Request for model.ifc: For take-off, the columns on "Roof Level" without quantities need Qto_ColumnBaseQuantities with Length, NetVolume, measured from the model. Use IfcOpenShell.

First a look at what the model holds.

```python
import ifcopenshell
import ifcopenshell.util.element
import ifcopenshell.util.unit

model = ifcopenshell.open("model.ifc")
print(model.schema)
for unit_type in ("LENGTHUNIT", "AREAUNIT", "VOLUMEUNIT"):
    print(unit_type, ifcopenshell.util.unit.calculate_unit_scale(model, unit_type))
storey = next(s for s in model.by_type("IfcBuildingStorey") if s.Name == "Roof Level")
columns = [e for e in ifcopenshell.util.element.get_decomposition(storey) if e.is_a("IfcColumn")]
for e in sorted(columns, key=lambda e: e.id()):
    print(e.id(), e.is_a(), e.Name, list(ifcopenshell.util.element.get_psets(e, qtos_only=True)), sep=" | ")
```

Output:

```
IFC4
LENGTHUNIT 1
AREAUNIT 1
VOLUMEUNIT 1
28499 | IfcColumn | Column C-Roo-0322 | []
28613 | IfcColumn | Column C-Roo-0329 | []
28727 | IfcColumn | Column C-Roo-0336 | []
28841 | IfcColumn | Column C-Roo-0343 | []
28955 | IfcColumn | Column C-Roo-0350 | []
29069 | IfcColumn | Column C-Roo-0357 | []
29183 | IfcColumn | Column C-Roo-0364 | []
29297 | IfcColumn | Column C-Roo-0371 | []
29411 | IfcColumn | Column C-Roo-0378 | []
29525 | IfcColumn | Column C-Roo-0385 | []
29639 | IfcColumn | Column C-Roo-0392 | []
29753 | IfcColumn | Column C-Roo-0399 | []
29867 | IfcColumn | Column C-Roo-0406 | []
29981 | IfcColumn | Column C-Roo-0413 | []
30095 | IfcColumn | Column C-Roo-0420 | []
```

```python
import ifcopenshell
import ifcopenshell.api.pset
import ifcopenshell.geom
import ifcopenshell.util.element
import ifcopenshell.util.shape
import ifcopenshell.util.unit

model = ifcopenshell.open("model.ifc")
unit_scale = ifcopenshell.util.unit.calculate_unit_scale(model)
volume_scale = ifcopenshell.util.unit.calculate_unit_scale(model, "VOLUMEUNIT")
settings = ifcopenshell.geom.settings()

storey = next(s for s in model.by_type("IfcBuildingStorey") if s.Name == "Roof Level")
columns = [e for e in ifcopenshell.util.element.get_decomposition(storey) if e.is_a("IfcColumn")]

for e in sorted(columns, key=lambda e: e.id()):
    if ifcopenshell.util.element.get_psets(e, qtos_only=True, should_inherit=False):
        continue
    # Geometry comes back in metres, in the element's own axes.
    shape = ifcopenshell.geom.create_shape(settings, e)
    values = {
        "Length": ifcopenshell.util.shape.get_z(shape.geometry) / unit_scale,
        "NetVolume": ifcopenshell.util.shape.get_volume(shape.geometry) / volume_scale,
    }
    qto = ifcopenshell.api.pset.add_qto(model, product=e, name="Qto_ColumnBaseQuantities")
    ifcopenshell.api.pset.edit_qto(model, qto=qto, properties=values)
    print(e.id(), {k: round(v, 3) for k, v in values.items()})

model.write("model_rev.ifc")
```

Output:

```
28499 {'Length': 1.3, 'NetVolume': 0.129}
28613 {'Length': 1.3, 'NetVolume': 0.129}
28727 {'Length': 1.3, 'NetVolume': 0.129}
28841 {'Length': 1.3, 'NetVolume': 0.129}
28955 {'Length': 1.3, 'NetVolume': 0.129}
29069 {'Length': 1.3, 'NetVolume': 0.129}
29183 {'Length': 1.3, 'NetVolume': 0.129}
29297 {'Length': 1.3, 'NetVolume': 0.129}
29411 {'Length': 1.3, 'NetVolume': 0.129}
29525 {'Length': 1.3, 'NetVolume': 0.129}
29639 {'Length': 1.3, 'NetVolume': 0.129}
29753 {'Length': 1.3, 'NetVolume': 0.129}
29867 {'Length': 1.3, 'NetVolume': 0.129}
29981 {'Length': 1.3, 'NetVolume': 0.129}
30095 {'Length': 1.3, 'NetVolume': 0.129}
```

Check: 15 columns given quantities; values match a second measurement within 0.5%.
